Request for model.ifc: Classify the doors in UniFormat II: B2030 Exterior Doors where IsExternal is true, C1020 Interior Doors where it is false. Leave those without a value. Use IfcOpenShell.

First a look at what the model holds.

```python
import ifcopenshell
import ifcopenshell.util.element

model = ifcopenshell.open("model.ifc")
print(model.schema)
print("classifications:", [c.Name for c in model.by_type("IfcClassification")])
values = [ifcopenshell.util.element.get_pset(e, "Pset_DoorCommon", "IsExternal") for e in model.by_type("IfcDoor")]
for value in (True, False, None):
    print("IsExternal", value, values.count(value))
```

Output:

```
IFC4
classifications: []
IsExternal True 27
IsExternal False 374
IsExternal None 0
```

```python
import ifcopenshell
import ifcopenshell.api.classification
import ifcopenshell.util.element

model = ifcopenshell.open("model.ifc")

system = ifcopenshell.api.classification.add_classification(model, classification="UniFormat II")

doors = model.by_type("IfcDoor")
external = {e: ifcopenshell.util.element.get_pset(e, "Pset_DoorCommon", "IsExternal") for e in doors}
for flag, code, name in ((True, "B2030", "Exterior Doors"), (False, "C1020", "Interior Doors")):
    products = [e for e in doors if external[e] is flag]
    ifcopenshell.api.classification.add_reference(
        model, products=products, classification=system, identification=code, name=name
    )
    print(code, len(products))

model.write("model_edited.ifc")
```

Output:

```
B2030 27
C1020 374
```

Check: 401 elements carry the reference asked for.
